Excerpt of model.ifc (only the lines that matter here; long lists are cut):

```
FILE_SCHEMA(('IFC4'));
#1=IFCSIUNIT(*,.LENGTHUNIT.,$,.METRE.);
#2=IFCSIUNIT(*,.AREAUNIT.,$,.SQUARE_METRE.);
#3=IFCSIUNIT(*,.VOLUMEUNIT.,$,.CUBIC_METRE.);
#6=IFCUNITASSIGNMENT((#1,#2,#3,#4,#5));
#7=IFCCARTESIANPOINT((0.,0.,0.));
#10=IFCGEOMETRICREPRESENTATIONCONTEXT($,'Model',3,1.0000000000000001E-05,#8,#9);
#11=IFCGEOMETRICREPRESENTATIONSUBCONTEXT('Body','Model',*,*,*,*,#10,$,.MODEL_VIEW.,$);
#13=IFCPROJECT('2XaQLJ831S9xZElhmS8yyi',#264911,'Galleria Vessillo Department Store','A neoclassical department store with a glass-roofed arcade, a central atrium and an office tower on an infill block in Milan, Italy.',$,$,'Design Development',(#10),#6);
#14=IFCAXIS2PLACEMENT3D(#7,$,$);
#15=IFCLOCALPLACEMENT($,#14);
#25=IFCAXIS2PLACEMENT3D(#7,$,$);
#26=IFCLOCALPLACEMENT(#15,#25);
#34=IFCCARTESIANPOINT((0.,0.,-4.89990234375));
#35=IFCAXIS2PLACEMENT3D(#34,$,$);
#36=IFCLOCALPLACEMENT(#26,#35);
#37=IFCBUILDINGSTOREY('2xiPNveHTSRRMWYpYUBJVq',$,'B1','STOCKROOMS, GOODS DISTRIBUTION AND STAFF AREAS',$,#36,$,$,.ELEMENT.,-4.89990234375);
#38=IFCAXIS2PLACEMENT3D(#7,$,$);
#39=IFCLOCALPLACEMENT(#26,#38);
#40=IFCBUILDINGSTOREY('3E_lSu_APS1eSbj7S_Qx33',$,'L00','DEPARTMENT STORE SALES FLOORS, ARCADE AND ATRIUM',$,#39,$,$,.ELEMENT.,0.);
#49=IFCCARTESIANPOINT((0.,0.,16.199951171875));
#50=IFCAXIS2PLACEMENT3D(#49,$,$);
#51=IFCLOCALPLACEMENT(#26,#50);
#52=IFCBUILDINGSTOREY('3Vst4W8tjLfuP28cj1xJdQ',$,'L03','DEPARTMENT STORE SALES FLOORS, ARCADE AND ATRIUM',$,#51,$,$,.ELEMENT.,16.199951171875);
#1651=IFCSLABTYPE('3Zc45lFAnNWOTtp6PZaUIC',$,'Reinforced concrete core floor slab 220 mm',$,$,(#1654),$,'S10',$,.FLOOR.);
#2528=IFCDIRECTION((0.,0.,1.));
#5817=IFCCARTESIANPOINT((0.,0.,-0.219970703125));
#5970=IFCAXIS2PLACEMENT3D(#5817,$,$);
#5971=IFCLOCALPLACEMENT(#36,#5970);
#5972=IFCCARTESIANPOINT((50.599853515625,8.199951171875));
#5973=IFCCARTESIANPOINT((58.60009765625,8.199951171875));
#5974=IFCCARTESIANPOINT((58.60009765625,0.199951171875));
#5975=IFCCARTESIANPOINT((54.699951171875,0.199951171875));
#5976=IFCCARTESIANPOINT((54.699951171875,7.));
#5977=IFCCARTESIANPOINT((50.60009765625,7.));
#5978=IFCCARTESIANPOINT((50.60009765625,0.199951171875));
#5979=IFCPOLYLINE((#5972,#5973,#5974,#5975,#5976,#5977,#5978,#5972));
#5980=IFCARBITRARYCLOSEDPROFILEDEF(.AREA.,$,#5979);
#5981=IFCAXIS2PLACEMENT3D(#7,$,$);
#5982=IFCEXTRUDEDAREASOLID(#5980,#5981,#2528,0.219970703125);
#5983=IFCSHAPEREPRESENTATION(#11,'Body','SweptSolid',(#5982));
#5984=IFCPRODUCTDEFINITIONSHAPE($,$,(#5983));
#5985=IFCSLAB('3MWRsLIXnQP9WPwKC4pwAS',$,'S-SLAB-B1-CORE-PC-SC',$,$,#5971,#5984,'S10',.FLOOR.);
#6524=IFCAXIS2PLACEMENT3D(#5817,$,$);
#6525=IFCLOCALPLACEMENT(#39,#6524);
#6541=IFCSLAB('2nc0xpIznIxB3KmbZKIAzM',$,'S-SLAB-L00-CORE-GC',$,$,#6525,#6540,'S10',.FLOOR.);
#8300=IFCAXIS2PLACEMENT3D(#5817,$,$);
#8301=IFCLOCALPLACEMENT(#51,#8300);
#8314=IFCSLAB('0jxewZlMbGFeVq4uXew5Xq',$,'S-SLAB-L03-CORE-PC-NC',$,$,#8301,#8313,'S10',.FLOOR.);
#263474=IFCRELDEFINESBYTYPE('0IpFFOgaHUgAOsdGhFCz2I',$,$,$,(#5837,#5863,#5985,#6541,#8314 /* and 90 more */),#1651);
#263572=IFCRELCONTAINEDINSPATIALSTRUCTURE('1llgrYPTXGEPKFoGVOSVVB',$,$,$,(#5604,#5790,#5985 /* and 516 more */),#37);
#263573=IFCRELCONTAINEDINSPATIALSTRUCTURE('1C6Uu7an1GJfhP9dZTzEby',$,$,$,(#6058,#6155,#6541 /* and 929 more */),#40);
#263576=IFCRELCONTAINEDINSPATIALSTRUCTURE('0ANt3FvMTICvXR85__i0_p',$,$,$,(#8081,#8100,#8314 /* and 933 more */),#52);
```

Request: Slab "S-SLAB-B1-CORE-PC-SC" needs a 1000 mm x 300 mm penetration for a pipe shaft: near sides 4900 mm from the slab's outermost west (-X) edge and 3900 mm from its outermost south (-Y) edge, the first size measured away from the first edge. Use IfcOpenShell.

```python
import numpy as np
import ifcopenshell
import ifcopenshell.api.feature
import ifcopenshell.api.geometry
import ifcopenshell.api.root
import ifcopenshell.geom
import ifcopenshell.util.placement
import ifcopenshell.util.representation
import ifcopenshell.util.shape
import ifcopenshell.util.unit

model = ifcopenshell.open("model.ifc")
unit_scale = ifcopenshell.util.unit.calculate_unit_scale(model)
settings = ifcopenshell.geom.settings()


def volume(element):
    """Net volume in cubic metres, openings subtracted."""
    shape = ifcopenshell.geom.create_shape(settings, element)
    return ifcopenshell.util.shape.get_volume(shape.geometry)


slab = model.by_guid("3MWRsLIXnQP9WPwKC4pwAS")
before = volume(slab)

# Extent in the slab's own axes, in metres. The edges named are its -X and -Y sides.
slab_shape = ifcopenshell.geom.create_shape(settings, slab)
vertices = ifcopenshell.util.shape.get_vertices(slab_shape.geometry)
x_min, y_min, bottom = vertices.min(axis=0)
top = vertices[:, 2].max()

opening = ifcopenshell.api.root.create_entity(model, ifc_class="IfcOpeningElement", name="Pipe shaft opening", predefined_type="OPENING")
context = ifcopenshell.util.representation.get_context(model, "Model", "Body", "MODEL_VIEW")
width, depth = 1, 0.3
outline = [(0.0, 0.0), (width, 0.0), (width, depth), (0.0, depth), (0.0, 0.0)]
# Overshoot both faces by 50 mm so the cut is clean.
shape = ifcopenshell.api.geometry.add_slab_representation(
    model, context=context, depth=top - bottom + 0.1, polyline=outline
)
ifcopenshell.api.geometry.assign_representation(model, product=opening, representation=shape)

matrix = ifcopenshell.util.placement.get_local_placement(slab.ObjectPlacement)
matrix[:, 3] = matrix @ np.append(np.array([x_min + 4.9, y_min + 3.9, bottom - 0.05]) / unit_scale, 1.0)
ifcopenshell.api.geometry.edit_object_placement(model, product=opening, matrix=matrix, is_si=False)
ifcopenshell.api.feature.add_feature(model, feature=opening, element=slab)

after = volume(slab)

print(f"slab volume {before:.3f} -> {after:.3f} m3")

model.write("model_edited.ifc")
```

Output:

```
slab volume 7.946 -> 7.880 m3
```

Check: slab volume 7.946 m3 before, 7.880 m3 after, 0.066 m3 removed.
